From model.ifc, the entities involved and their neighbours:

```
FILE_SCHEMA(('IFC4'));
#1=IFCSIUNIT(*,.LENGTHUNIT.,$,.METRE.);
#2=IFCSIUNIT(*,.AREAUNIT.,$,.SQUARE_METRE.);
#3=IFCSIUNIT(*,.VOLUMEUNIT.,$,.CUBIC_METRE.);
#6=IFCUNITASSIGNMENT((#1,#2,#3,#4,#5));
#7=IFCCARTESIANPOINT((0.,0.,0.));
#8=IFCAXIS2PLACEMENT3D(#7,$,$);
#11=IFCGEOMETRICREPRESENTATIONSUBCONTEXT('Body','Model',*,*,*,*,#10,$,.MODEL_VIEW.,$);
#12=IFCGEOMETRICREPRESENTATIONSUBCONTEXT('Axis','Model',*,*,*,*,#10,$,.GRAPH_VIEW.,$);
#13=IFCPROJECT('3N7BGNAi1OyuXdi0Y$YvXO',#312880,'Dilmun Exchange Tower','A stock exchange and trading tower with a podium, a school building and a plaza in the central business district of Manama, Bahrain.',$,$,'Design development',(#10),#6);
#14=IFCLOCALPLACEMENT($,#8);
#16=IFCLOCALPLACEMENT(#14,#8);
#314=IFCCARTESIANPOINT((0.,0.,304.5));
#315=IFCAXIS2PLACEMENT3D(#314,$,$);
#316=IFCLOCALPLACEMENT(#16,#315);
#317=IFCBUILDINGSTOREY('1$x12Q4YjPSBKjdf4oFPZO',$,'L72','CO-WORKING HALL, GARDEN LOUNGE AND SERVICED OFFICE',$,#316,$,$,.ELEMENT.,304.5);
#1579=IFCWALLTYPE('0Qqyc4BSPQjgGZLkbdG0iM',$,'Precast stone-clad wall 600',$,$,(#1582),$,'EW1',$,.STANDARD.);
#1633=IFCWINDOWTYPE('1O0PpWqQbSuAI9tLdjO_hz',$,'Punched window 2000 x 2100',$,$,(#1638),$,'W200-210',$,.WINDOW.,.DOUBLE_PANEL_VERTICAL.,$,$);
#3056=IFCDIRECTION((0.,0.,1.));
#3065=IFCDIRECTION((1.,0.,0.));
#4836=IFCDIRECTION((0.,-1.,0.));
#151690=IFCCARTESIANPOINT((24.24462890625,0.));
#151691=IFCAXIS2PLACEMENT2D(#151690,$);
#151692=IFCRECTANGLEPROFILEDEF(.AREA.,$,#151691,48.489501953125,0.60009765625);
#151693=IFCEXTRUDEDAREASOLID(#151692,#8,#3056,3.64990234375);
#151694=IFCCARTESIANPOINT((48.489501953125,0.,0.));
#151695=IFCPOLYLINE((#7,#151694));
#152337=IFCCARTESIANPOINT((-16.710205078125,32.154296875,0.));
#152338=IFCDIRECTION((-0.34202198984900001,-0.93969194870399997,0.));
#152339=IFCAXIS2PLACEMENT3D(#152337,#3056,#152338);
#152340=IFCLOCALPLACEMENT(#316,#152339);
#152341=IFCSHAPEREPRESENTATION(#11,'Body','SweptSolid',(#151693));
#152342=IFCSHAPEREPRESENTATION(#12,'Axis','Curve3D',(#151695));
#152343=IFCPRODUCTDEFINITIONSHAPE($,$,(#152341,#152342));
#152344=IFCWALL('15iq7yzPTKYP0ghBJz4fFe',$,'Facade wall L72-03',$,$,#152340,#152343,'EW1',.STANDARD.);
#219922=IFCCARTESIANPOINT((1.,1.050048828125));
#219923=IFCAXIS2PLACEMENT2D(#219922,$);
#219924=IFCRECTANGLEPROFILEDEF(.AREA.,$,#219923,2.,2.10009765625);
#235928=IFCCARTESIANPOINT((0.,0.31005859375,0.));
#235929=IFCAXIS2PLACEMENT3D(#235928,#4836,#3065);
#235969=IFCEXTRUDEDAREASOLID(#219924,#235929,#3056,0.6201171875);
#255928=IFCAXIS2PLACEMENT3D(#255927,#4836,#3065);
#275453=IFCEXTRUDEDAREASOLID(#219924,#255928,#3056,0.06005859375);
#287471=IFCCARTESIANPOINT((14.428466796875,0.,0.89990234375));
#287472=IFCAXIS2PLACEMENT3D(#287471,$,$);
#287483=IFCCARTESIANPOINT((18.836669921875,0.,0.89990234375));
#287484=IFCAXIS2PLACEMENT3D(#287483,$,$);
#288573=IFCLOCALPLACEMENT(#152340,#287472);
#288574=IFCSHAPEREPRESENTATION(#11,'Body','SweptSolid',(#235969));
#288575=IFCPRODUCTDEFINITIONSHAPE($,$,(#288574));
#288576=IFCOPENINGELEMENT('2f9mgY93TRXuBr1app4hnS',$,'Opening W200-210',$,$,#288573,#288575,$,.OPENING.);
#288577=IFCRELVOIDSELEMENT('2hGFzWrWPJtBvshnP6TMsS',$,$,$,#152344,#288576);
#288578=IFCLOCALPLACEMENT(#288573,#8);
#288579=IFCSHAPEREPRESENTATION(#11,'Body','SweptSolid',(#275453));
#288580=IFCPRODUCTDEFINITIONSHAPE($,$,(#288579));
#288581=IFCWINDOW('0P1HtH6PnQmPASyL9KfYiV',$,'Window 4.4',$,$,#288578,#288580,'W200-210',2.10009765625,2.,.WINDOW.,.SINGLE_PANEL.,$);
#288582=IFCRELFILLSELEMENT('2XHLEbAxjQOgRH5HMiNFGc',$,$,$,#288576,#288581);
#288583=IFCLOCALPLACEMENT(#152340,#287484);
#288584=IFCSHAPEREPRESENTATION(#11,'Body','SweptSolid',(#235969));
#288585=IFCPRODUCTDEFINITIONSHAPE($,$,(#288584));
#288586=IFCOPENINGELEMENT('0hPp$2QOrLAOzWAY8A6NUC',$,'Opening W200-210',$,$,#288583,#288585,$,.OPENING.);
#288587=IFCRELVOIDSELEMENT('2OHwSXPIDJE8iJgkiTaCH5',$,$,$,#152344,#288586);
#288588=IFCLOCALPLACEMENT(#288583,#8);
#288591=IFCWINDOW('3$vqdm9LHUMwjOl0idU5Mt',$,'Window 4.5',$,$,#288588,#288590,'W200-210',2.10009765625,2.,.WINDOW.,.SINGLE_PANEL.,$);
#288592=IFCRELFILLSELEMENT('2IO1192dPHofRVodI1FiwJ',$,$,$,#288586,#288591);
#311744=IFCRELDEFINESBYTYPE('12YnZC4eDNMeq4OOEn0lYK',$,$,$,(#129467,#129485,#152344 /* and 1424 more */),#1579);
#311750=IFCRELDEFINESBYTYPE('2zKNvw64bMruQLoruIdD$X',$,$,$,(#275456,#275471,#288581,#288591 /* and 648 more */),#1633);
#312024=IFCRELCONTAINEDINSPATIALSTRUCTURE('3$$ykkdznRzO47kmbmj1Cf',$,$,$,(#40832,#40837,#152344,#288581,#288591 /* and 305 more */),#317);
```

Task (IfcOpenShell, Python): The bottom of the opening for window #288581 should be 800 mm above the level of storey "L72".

```python
import numpy as np
import ifcopenshell
import ifcopenshell.api.geometry
import ifcopenshell.geom
import ifcopenshell.util.element
import ifcopenshell.util.placement
import ifcopenshell.util.shape
import ifcopenshell.util.unit

model = ifcopenshell.open("model.ifc")
unit_scale = ifcopenshell.util.unit.calculate_unit_scale(model)

window = model.by_guid("0P1HtH6PnQmPASyL9KfYiV")
opening = window.FillsVoids[0].RelatingOpeningElement
storey = ifcopenshell.util.element.get_container(window, ifc_class="IfcBuildingStorey")
level = ifcopenshell.util.placement.get_local_placement(storey.ObjectPlacement)[2, 3]

# The opening's origin need not be at the sill, so measure its lowest point.
shape = ifcopenshell.geom.create_shape(ifcopenshell.geom.settings(), opening)
bottom = ifcopenshell.util.shape.get_shape_bottom_elevation(shape, shape.geometry) / unit_scale
dz = level + 0.8 / unit_scale - bottom

shift = np.array([0.0, 0.0, dz])
# The window is placed relative to its opening, so it follows when the opening moves.
matrix = ifcopenshell.util.placement.get_local_placement(opening.ObjectPlacement)
matrix[:3, 3] += shift
ifcopenshell.api.geometry.edit_object_placement(
    model, product=opening, matrix=matrix, is_si=False, should_transform_children=True
)

print(f"moved by {dz * unit_scale:+.3f} m")

model.write("model-out.ifc")
```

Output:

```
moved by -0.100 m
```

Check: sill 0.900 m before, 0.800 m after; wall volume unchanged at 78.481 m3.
